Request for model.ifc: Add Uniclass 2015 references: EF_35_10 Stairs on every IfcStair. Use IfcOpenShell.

First a look at what the model holds.

```python
import ifcopenshell

model = ifcopenshell.open("model.ifc")
print(model.schema)
print("classifications:", [c.Name for c in model.by_type("IfcClassification")])
for ifc_class in ("IfcDoor", "IfcRoof", "IfcStair", "IfcWall", "IfcWindow"):
    print(ifc_class, len(model.by_type(ifc_class)))
```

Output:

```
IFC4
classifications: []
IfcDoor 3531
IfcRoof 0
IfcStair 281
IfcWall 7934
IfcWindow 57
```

```python
import ifcopenshell
import ifcopenshell.api.classification

model = ifcopenshell.open("model.ifc")

system = ifcopenshell.api.classification.add_classification(model, classification="Uniclass 2015")

codes = {
    "IfcStair": ("EF_35_10", "Stairs"),
}
for ifc_class, (code, name) in codes.items():
    products = model.by_type(ifc_class)
    ifcopenshell.api.classification.add_reference(
        model, products=products, classification=system, identification=code, name=name
    )
    print(code, len(products))

model.write("model_rev.ifc")
```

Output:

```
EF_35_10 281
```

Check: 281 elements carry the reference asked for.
